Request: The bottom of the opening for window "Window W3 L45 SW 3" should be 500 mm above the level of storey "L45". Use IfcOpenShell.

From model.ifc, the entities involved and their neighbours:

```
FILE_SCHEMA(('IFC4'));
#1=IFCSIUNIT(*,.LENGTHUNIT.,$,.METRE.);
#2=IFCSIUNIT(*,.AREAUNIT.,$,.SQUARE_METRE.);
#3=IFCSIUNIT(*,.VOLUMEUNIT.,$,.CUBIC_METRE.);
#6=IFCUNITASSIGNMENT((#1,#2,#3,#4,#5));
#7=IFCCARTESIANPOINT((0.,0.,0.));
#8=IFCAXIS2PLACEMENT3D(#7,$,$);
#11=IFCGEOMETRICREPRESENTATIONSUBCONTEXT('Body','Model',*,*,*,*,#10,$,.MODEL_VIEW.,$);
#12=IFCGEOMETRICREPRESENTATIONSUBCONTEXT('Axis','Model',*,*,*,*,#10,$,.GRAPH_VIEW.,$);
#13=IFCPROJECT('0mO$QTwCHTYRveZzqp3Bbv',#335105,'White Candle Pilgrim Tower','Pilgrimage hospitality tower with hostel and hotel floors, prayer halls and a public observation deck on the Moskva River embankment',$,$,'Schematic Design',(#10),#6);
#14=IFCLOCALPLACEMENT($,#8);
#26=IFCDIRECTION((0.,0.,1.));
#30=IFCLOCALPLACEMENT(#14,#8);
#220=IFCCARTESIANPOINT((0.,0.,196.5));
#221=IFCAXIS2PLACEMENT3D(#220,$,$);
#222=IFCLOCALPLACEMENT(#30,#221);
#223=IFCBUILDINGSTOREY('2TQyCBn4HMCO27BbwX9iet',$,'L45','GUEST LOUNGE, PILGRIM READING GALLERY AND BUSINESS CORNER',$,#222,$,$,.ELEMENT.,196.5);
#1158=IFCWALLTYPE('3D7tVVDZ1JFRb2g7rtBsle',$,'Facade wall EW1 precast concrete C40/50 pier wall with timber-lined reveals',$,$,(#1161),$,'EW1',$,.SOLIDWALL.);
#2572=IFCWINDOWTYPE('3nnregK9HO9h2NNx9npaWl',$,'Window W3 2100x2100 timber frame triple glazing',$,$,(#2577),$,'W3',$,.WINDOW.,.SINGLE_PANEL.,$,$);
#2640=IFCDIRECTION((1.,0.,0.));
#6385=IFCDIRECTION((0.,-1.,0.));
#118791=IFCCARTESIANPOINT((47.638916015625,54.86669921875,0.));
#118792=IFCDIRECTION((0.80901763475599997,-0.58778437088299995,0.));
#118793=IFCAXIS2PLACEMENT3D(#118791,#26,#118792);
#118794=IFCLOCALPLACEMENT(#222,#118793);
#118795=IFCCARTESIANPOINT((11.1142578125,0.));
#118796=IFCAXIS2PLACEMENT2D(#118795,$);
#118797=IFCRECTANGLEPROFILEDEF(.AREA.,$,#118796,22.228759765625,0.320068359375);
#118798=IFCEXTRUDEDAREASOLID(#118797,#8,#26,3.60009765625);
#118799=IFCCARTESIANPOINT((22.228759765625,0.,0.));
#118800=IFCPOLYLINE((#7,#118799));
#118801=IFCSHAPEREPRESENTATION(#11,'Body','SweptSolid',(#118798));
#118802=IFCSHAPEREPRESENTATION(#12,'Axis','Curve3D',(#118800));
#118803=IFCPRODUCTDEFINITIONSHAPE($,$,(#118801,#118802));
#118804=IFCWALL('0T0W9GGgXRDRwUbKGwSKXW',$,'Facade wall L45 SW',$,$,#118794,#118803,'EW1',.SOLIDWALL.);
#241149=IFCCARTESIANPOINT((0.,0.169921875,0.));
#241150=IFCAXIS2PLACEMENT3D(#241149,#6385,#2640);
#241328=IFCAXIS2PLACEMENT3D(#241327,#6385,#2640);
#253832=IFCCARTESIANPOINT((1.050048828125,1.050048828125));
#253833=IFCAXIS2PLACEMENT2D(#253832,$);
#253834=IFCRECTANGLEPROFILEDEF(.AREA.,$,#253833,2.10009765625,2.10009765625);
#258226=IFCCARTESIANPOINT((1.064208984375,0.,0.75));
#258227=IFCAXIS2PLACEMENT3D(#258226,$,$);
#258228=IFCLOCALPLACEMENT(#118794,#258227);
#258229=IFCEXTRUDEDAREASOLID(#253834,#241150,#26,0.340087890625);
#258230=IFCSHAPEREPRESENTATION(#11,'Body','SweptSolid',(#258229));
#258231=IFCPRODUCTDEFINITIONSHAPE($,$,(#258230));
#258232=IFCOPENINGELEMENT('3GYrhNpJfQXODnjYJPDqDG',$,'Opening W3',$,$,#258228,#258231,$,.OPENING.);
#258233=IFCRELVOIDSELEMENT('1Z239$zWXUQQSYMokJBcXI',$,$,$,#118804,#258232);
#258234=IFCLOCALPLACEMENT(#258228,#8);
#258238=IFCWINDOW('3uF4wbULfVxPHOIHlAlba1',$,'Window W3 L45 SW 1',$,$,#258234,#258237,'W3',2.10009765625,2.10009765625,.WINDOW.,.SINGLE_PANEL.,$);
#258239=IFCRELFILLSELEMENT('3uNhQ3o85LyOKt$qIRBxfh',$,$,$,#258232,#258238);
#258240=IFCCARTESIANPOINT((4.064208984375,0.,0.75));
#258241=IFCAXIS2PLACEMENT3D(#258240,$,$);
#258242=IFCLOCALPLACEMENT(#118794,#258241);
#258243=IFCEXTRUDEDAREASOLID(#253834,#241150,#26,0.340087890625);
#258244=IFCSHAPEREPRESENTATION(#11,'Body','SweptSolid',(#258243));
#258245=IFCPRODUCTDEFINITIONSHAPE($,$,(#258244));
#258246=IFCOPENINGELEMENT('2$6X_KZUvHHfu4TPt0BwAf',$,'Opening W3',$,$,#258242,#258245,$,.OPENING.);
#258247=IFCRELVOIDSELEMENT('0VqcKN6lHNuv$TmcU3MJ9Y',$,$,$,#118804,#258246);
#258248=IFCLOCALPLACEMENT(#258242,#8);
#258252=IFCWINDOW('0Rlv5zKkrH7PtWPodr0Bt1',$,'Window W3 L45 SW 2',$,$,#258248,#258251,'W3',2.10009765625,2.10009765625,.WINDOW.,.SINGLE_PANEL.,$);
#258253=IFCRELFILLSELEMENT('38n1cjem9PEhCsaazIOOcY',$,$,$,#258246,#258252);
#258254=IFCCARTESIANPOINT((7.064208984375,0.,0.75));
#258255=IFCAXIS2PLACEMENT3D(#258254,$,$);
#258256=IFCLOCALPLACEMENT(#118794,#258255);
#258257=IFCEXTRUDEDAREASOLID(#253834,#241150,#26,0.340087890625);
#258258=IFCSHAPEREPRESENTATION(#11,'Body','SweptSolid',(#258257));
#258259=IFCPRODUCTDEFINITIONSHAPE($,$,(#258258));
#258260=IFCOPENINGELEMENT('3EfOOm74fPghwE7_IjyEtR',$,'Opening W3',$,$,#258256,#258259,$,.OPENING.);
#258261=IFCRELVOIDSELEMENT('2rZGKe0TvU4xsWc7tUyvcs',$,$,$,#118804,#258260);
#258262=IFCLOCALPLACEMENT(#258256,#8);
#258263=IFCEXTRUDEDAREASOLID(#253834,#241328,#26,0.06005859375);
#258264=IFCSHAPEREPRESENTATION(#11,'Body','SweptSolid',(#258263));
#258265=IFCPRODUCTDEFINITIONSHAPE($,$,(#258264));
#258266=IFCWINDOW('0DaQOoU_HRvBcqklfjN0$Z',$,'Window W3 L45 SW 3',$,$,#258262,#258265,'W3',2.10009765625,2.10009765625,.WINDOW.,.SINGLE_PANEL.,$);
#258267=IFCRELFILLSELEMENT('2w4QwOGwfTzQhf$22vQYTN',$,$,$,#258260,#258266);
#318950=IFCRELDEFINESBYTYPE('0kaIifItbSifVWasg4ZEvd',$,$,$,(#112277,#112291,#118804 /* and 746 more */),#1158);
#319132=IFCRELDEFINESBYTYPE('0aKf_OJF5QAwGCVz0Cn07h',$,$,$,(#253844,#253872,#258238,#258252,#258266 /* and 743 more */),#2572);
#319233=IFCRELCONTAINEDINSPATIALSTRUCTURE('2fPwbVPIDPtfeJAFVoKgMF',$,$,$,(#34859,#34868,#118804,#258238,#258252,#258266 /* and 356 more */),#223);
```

```python
import numpy as np
import ifcopenshell
import ifcopenshell.api.geometry
import ifcopenshell.geom
import ifcopenshell.util.element
import ifcopenshell.util.placement
import ifcopenshell.util.shape
import ifcopenshell.util.unit

model = ifcopenshell.open("model.ifc")
unit_scale = ifcopenshell.util.unit.calculate_unit_scale(model)

window = model.by_id(258266)
opening = window.FillsVoids[0].RelatingOpeningElement
storey = ifcopenshell.util.element.get_container(window, ifc_class="IfcBuildingStorey")
level = ifcopenshell.util.placement.get_local_placement(storey.ObjectPlacement)[2, 3]

# The opening's origin need not be at the sill, so measure its lowest point.
shape = ifcopenshell.geom.create_shape(ifcopenshell.geom.settings(), opening)
bottom = ifcopenshell.util.shape.get_shape_bottom_elevation(shape, shape.geometry) / unit_scale
dz = level + 0.5 / unit_scale - bottom

shift = np.array([0.0, 0.0, dz])
# The window is placed relative to its opening, so it follows when the opening moves.
matrix = ifcopenshell.util.placement.get_local_placement(opening.ObjectPlacement)
matrix[:3, 3] += shift
ifcopenshell.api.geometry.edit_object_placement(
    model, product=opening, matrix=matrix, is_si=False, should_transform_children=True
)

print(f"moved by {dz * unit_scale:+.3f} m")

model.write("model_updated.ifc")
```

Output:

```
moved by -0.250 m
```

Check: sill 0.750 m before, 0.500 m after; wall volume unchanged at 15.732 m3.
